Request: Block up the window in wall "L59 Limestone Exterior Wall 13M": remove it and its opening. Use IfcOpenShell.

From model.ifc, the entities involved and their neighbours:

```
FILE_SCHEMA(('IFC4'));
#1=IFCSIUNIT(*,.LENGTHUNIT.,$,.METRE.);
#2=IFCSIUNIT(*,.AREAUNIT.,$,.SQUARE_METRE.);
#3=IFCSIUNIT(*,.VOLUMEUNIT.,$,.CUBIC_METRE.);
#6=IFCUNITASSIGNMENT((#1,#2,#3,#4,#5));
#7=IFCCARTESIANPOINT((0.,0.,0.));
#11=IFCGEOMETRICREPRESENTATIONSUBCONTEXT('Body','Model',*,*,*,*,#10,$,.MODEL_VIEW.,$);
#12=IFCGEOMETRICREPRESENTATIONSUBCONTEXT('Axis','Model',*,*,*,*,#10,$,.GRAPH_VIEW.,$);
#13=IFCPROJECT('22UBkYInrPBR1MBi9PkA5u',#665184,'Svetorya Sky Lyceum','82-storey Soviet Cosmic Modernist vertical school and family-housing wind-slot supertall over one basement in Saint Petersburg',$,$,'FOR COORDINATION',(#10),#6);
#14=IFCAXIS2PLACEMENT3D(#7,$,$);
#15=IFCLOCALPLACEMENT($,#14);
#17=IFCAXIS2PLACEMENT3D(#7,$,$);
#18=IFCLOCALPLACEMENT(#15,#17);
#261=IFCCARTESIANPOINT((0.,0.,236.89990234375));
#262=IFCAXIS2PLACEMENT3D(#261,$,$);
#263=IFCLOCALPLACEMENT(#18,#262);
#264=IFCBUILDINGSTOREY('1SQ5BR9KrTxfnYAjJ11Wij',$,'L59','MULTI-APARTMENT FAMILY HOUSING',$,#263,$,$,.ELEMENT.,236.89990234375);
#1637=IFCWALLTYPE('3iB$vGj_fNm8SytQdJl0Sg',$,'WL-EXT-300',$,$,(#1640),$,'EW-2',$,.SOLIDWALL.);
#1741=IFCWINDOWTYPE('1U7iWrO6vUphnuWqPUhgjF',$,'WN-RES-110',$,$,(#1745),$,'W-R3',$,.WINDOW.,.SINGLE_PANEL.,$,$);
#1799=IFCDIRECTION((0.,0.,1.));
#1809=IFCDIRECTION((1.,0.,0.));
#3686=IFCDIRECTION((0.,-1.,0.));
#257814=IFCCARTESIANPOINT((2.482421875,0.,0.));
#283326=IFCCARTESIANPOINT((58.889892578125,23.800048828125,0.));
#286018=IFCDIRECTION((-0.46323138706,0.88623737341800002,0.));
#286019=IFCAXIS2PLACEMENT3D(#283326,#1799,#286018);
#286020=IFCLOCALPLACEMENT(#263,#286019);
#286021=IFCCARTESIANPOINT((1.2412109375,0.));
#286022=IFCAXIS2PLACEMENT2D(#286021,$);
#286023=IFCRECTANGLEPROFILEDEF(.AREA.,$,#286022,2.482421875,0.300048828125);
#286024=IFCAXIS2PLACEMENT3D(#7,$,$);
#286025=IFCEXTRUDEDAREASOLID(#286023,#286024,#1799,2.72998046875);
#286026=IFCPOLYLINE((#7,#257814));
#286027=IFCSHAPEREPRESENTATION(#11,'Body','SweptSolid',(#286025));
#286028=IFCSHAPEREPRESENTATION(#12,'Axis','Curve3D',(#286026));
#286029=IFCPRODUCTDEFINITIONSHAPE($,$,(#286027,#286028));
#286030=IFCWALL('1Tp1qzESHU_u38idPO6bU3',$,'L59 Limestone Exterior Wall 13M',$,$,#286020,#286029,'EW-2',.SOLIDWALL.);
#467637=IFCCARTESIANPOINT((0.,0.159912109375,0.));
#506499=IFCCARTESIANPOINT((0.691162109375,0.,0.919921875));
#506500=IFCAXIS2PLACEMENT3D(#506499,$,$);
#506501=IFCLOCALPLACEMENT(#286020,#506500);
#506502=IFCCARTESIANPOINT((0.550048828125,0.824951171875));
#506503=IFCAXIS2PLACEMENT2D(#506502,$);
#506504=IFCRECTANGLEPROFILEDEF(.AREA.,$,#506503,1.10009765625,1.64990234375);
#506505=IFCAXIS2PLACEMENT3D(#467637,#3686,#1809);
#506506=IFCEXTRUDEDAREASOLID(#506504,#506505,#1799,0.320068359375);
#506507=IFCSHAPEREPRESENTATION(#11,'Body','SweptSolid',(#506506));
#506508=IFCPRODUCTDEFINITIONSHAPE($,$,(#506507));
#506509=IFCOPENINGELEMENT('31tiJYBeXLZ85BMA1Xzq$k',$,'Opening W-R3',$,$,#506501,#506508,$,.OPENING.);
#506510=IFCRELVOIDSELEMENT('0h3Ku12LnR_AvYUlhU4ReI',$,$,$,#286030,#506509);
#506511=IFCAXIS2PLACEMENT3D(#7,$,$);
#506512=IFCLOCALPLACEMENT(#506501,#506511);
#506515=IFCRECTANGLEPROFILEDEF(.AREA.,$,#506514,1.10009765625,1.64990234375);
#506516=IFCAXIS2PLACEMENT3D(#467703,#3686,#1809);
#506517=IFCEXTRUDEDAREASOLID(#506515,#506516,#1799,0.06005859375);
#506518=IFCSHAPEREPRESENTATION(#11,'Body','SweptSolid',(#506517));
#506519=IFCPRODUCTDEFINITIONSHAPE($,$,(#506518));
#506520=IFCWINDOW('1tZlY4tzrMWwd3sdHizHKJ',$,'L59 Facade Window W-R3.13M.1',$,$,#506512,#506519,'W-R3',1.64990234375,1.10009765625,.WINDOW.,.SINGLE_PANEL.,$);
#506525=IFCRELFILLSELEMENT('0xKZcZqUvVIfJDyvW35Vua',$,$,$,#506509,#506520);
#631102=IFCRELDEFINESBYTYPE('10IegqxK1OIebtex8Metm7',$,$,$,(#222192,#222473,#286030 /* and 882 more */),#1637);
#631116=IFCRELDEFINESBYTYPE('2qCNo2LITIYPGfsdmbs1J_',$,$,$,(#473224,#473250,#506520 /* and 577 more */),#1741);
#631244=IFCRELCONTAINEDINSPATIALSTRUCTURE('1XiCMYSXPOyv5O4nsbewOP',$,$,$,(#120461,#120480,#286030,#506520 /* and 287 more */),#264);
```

```python
import ifcopenshell
import ifcopenshell.api.feature
import ifcopenshell.api.root
import ifcopenshell.geom
import ifcopenshell.util.shape

model = ifcopenshell.open("model.ifc")
settings = ifcopenshell.geom.settings()


def volume(element):
    """Net volume in cubic metres, openings subtracted."""
    shape = ifcopenshell.geom.create_shape(settings, element)
    return ifcopenshell.util.shape.get_volume(shape.geometry)


window = model.by_guid("1tZlY4tzrMWwd3sdHizHKJ")
opening = window.FillsVoids[0].RelatingOpeningElement
wall = opening.VoidsElements[0].RelatingBuildingElement
before = volume(wall)

ifcopenshell.api.root.remove_product(model, product=window)
ifcopenshell.api.feature.remove_feature(model, feature=opening)

after = volume(wall)

print(f"wall volume {before:.3f} -> {after:.3f} m3")

model.write("model_edited.ifc")
```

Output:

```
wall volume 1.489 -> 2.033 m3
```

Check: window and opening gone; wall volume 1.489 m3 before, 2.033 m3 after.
